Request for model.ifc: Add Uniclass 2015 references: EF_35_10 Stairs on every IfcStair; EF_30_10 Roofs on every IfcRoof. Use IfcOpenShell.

First a look at what the model holds.

```python
import ifcopenshell

model = ifcopenshell.open("model.ifc")
print(model.schema)
print("classifications:", [c.Name for c in model.by_type("IfcClassification")])
for ifc_class in ("IfcDoor", "IfcRoof", "IfcStair", "IfcWall", "IfcWindow"):
    print(ifc_class, len(model.by_type(ifc_class)))
```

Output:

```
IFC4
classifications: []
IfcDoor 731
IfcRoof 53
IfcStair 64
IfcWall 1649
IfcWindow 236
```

```python
import ifcopenshell
import ifcopenshell.api.classification

model = ifcopenshell.open("model.ifc")

system = ifcopenshell.api.classification.add_classification(model, classification="Uniclass 2015")

codes = {
    "IfcStair": ("EF_35_10", "Stairs"),
    "IfcRoof": ("EF_30_10", "Roofs"),
}
for ifc_class, (code, name) in codes.items():
    products = model.by_type(ifc_class)
    ifcopenshell.api.classification.add_reference(
        model, products=products, classification=system, identification=code, name=name
    )
    print(code, len(products))

model.write("model_v2.ifc")
```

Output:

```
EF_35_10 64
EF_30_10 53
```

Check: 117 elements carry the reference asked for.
